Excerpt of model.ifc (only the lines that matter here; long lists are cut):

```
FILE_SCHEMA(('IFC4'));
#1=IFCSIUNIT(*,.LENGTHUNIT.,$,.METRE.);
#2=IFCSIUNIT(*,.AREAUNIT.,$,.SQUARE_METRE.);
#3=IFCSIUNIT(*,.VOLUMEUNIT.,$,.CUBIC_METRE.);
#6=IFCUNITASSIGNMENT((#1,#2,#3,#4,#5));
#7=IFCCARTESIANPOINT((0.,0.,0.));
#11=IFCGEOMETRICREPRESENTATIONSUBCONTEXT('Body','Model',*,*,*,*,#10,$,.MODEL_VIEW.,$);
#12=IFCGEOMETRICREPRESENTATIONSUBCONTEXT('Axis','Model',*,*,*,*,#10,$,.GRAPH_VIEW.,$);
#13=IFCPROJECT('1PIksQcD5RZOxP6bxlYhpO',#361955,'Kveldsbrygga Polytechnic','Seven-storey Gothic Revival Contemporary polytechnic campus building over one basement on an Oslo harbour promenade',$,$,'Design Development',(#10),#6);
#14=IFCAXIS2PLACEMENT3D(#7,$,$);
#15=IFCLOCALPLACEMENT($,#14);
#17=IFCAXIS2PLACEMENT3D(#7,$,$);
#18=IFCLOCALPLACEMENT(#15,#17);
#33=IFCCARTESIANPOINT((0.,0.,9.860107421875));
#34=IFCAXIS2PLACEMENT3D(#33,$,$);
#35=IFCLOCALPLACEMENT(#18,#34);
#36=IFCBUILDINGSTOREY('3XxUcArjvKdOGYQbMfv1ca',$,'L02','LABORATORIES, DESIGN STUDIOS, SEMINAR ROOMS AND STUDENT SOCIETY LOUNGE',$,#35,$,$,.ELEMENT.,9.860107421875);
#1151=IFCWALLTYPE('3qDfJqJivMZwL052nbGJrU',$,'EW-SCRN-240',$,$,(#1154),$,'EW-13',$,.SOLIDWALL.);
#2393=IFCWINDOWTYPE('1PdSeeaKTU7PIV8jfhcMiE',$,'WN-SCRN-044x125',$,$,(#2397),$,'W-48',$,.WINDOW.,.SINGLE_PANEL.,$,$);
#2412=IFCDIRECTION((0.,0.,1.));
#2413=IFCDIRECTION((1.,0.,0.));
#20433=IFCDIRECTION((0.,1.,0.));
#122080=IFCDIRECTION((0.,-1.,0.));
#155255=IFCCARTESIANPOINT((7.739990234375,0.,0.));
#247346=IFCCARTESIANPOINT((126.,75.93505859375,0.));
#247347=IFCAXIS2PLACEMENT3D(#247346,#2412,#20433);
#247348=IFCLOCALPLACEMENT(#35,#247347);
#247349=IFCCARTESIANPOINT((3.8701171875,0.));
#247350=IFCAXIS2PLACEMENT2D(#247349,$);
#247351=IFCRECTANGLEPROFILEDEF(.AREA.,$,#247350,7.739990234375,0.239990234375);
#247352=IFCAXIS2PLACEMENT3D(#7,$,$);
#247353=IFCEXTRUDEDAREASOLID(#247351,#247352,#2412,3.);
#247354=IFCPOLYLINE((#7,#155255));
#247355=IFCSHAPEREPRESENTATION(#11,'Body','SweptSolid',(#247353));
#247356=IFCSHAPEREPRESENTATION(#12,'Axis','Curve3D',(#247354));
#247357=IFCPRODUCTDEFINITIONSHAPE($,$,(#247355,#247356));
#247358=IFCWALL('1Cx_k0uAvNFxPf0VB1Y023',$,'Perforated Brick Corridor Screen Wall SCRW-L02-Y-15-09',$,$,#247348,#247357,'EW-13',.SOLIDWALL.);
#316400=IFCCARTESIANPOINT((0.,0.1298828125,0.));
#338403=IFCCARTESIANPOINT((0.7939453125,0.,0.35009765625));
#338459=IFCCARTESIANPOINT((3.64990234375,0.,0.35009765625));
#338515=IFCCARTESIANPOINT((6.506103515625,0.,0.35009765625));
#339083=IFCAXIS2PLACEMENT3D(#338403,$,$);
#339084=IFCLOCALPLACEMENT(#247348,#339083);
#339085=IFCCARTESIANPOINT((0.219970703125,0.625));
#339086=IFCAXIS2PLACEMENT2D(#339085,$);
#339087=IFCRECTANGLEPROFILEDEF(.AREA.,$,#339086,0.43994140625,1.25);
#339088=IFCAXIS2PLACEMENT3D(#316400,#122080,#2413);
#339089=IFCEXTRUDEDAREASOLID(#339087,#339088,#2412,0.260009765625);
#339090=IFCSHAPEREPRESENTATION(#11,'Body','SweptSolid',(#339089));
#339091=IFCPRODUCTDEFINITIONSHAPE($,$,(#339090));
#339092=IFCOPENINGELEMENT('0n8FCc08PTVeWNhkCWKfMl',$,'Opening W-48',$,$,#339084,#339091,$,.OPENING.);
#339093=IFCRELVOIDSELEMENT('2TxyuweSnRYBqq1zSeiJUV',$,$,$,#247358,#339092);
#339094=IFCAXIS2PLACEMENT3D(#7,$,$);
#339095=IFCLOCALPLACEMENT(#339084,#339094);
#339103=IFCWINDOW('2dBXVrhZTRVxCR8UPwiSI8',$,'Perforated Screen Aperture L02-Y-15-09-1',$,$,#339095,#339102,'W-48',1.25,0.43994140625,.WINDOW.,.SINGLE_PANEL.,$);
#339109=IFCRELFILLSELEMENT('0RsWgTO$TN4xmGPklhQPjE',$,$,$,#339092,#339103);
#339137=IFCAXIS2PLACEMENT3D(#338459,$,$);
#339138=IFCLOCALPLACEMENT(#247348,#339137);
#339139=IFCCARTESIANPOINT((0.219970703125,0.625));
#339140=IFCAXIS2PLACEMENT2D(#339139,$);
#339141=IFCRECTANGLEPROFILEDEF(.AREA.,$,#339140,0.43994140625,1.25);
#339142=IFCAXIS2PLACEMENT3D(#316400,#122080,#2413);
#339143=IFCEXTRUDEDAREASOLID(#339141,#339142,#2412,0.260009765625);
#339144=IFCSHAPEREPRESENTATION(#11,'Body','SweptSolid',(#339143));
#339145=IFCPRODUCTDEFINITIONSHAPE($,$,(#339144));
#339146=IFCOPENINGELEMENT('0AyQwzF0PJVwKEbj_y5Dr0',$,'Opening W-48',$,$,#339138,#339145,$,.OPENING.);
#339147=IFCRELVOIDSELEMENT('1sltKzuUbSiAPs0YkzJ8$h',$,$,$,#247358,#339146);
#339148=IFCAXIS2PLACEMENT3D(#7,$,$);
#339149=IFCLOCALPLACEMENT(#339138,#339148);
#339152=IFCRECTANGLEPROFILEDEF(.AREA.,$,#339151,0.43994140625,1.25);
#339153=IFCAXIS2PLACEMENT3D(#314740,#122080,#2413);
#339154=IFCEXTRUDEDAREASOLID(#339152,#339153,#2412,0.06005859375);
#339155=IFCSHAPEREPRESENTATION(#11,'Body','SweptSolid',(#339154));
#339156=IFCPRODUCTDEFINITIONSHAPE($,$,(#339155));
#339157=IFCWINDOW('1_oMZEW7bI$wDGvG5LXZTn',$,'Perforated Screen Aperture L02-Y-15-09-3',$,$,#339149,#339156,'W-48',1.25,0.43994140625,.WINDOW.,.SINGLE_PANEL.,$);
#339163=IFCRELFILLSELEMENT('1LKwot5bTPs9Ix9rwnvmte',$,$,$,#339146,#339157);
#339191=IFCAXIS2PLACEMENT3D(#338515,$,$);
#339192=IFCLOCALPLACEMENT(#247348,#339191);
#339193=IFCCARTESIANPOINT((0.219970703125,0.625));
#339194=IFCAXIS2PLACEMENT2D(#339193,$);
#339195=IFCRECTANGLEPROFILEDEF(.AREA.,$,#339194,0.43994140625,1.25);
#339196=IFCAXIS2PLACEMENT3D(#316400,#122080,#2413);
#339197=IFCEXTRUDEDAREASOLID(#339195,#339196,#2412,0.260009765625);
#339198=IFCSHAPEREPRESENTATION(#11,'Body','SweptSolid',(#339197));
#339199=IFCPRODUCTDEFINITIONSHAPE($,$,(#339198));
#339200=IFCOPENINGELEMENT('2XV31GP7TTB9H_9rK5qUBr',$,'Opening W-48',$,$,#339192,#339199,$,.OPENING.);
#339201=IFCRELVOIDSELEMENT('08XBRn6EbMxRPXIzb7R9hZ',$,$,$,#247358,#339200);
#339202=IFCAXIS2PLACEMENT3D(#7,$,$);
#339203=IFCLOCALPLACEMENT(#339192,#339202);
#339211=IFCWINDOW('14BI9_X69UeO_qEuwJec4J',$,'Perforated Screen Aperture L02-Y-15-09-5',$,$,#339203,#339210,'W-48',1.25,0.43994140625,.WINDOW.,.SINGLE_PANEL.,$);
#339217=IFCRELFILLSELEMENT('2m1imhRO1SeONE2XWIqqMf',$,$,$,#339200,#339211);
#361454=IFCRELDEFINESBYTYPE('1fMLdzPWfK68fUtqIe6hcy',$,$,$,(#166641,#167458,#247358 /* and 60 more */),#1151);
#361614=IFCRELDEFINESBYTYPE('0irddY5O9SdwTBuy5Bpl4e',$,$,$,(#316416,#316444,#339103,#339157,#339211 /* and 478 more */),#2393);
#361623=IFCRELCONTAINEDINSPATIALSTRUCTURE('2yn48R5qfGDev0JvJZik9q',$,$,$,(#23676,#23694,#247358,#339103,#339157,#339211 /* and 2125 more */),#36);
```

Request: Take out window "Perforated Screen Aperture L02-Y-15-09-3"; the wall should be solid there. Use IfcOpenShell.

```python
import ifcopenshell
import ifcopenshell.api.feature
import ifcopenshell.api.root
import ifcopenshell.geom
import ifcopenshell.util.shape

model = ifcopenshell.open("model.ifc")
settings = ifcopenshell.geom.settings()


def volume(element):
    """Net volume in cubic metres, openings subtracted."""
    shape = ifcopenshell.geom.create_shape(settings, element)
    return ifcopenshell.util.shape.get_volume(shape.geometry)


window = model.by_id(339157)
opening = window.FillsVoids[0].RelatingOpeningElement
wall = opening.VoidsElements[0].RelatingBuildingElement
before = volume(wall)

ifcopenshell.api.root.remove_product(model, product=window)
ifcopenshell.api.feature.remove_feature(model, feature=opening)

after = volume(wall)

print(f"wall volume {before:.3f} -> {after:.3f} m3")

model.write("model_updated.ifc")
```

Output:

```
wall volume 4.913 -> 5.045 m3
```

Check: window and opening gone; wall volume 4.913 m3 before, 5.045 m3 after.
